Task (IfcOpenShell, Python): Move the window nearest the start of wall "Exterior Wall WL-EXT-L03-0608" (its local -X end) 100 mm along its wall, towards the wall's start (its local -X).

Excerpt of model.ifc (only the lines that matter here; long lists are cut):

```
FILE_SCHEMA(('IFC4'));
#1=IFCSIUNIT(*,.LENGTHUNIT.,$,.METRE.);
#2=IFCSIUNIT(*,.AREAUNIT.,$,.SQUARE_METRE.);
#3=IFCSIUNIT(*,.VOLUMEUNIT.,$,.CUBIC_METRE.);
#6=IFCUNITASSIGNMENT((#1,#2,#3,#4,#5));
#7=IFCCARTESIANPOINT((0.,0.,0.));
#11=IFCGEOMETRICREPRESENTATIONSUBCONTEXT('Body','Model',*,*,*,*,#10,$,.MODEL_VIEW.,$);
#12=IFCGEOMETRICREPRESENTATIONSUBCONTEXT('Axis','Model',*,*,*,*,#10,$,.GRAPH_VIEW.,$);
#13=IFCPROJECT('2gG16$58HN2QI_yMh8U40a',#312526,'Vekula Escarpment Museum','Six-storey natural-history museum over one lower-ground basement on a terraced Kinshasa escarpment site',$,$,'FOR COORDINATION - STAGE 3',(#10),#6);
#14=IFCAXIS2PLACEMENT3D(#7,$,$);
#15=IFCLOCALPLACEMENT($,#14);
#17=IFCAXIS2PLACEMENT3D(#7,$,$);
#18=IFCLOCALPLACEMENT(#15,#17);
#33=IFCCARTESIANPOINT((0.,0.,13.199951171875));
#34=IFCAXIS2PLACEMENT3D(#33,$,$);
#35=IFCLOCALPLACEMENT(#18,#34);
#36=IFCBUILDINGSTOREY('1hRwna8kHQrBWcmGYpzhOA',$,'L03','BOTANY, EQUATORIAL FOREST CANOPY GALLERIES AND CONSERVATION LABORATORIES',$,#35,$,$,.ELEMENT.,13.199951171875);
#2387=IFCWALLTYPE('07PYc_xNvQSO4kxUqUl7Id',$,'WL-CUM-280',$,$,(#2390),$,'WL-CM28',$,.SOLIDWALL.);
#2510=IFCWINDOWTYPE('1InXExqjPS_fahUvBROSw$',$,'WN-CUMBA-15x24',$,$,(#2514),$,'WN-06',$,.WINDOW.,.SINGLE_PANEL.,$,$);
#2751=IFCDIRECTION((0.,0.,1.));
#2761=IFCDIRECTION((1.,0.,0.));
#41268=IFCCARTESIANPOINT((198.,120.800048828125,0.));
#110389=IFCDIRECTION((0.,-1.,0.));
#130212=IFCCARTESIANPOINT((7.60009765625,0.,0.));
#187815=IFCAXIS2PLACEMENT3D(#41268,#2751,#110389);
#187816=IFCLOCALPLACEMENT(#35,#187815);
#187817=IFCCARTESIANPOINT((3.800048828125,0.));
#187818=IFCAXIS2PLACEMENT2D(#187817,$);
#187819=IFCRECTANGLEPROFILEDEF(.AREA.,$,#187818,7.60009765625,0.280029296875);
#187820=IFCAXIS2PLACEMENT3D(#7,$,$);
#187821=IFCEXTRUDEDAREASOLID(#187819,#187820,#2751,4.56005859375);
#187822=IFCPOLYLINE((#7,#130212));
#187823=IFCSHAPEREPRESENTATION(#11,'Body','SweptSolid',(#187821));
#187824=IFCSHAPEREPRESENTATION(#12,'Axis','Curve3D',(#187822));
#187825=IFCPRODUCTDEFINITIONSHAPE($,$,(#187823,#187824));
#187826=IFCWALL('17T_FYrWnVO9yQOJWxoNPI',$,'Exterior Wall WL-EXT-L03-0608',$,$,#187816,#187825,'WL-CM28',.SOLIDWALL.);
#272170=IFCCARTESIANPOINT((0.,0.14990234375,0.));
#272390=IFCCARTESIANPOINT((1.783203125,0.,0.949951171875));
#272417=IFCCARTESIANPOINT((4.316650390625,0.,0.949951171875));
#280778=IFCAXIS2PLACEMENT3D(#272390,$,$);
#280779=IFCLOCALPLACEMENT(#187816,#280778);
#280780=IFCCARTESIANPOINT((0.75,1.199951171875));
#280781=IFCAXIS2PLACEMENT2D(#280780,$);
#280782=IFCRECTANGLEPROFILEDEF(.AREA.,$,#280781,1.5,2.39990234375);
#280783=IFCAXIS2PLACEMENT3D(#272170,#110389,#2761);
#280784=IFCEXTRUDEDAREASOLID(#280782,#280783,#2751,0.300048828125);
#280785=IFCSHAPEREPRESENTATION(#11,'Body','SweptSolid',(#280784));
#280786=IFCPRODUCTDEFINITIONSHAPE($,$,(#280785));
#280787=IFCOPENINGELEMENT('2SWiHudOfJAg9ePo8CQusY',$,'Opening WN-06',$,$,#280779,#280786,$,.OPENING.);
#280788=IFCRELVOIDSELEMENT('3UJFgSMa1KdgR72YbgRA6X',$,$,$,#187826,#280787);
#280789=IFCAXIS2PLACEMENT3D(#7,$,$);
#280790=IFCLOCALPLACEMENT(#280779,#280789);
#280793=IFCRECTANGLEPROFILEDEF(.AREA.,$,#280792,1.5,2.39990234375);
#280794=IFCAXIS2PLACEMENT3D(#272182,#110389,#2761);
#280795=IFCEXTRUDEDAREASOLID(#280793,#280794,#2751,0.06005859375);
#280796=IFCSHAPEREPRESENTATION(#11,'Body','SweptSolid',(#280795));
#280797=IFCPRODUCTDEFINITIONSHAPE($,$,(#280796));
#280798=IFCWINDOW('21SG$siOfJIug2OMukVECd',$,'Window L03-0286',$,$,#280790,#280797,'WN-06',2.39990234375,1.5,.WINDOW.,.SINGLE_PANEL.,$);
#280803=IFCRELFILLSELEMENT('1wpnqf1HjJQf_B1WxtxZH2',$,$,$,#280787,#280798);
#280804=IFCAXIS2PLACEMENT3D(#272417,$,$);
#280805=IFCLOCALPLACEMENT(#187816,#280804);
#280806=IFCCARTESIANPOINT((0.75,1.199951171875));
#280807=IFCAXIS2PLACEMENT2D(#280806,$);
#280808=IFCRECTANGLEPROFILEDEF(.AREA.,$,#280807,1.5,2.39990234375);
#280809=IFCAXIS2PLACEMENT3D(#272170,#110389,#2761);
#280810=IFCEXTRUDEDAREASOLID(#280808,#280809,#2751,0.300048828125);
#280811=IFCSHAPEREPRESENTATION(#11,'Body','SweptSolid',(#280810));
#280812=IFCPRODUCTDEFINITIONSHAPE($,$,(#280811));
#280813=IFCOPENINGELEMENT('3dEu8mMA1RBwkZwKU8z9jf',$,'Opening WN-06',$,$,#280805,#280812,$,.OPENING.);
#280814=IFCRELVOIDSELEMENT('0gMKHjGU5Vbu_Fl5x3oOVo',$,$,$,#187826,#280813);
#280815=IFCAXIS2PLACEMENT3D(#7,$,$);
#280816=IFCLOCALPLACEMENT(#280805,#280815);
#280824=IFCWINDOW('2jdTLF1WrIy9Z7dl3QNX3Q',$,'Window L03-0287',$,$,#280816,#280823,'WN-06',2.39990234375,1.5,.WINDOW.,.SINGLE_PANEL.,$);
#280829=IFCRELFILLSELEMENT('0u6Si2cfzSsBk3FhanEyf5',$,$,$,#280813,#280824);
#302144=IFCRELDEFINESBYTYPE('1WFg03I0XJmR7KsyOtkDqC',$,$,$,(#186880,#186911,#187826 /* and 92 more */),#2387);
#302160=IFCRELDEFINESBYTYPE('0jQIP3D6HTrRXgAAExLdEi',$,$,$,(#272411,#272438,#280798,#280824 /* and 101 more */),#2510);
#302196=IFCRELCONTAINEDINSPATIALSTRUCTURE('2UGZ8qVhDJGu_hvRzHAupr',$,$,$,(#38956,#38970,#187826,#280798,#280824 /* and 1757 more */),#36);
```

```python
import ifcopenshell
import ifcopenshell.api.geometry
import ifcopenshell.util.placement
import ifcopenshell.util.unit

model = ifcopenshell.open("model.ifc")
unit_scale = ifcopenshell.util.unit.calculate_unit_scale(model)

window = model.by_guid("21SG$siOfJIug2OMukVECd")
opening = window.FillsVoids[0].RelatingOpeningElement
wall = opening.VoidsElements[0].RelatingBuildingElement

wall_matrix = ifcopenshell.util.placement.get_local_placement(wall.ObjectPlacement)
shift = wall_matrix[:3, 0] * -0.1 / unit_scale
before = ifcopenshell.util.placement.get_local_placement(window.ObjectPlacement)[:3, 3].copy()

# The window is placed relative to its opening, so it follows when the opening moves.
matrix = ifcopenshell.util.placement.get_local_placement(opening.ObjectPlacement)
matrix[:3, 3] += shift
ifcopenshell.api.geometry.edit_object_placement(
    model, product=opening, matrix=matrix, is_si=False, should_transform_children=True
)

after = ifcopenshell.util.placement.get_local_placement(window.ObjectPlacement)[:3, 3]
print("window moved by", (after - before).round(3) + 0.0)

model.write("model_v2.ifc")
```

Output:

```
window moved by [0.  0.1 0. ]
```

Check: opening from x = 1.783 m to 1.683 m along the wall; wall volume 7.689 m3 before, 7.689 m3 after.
